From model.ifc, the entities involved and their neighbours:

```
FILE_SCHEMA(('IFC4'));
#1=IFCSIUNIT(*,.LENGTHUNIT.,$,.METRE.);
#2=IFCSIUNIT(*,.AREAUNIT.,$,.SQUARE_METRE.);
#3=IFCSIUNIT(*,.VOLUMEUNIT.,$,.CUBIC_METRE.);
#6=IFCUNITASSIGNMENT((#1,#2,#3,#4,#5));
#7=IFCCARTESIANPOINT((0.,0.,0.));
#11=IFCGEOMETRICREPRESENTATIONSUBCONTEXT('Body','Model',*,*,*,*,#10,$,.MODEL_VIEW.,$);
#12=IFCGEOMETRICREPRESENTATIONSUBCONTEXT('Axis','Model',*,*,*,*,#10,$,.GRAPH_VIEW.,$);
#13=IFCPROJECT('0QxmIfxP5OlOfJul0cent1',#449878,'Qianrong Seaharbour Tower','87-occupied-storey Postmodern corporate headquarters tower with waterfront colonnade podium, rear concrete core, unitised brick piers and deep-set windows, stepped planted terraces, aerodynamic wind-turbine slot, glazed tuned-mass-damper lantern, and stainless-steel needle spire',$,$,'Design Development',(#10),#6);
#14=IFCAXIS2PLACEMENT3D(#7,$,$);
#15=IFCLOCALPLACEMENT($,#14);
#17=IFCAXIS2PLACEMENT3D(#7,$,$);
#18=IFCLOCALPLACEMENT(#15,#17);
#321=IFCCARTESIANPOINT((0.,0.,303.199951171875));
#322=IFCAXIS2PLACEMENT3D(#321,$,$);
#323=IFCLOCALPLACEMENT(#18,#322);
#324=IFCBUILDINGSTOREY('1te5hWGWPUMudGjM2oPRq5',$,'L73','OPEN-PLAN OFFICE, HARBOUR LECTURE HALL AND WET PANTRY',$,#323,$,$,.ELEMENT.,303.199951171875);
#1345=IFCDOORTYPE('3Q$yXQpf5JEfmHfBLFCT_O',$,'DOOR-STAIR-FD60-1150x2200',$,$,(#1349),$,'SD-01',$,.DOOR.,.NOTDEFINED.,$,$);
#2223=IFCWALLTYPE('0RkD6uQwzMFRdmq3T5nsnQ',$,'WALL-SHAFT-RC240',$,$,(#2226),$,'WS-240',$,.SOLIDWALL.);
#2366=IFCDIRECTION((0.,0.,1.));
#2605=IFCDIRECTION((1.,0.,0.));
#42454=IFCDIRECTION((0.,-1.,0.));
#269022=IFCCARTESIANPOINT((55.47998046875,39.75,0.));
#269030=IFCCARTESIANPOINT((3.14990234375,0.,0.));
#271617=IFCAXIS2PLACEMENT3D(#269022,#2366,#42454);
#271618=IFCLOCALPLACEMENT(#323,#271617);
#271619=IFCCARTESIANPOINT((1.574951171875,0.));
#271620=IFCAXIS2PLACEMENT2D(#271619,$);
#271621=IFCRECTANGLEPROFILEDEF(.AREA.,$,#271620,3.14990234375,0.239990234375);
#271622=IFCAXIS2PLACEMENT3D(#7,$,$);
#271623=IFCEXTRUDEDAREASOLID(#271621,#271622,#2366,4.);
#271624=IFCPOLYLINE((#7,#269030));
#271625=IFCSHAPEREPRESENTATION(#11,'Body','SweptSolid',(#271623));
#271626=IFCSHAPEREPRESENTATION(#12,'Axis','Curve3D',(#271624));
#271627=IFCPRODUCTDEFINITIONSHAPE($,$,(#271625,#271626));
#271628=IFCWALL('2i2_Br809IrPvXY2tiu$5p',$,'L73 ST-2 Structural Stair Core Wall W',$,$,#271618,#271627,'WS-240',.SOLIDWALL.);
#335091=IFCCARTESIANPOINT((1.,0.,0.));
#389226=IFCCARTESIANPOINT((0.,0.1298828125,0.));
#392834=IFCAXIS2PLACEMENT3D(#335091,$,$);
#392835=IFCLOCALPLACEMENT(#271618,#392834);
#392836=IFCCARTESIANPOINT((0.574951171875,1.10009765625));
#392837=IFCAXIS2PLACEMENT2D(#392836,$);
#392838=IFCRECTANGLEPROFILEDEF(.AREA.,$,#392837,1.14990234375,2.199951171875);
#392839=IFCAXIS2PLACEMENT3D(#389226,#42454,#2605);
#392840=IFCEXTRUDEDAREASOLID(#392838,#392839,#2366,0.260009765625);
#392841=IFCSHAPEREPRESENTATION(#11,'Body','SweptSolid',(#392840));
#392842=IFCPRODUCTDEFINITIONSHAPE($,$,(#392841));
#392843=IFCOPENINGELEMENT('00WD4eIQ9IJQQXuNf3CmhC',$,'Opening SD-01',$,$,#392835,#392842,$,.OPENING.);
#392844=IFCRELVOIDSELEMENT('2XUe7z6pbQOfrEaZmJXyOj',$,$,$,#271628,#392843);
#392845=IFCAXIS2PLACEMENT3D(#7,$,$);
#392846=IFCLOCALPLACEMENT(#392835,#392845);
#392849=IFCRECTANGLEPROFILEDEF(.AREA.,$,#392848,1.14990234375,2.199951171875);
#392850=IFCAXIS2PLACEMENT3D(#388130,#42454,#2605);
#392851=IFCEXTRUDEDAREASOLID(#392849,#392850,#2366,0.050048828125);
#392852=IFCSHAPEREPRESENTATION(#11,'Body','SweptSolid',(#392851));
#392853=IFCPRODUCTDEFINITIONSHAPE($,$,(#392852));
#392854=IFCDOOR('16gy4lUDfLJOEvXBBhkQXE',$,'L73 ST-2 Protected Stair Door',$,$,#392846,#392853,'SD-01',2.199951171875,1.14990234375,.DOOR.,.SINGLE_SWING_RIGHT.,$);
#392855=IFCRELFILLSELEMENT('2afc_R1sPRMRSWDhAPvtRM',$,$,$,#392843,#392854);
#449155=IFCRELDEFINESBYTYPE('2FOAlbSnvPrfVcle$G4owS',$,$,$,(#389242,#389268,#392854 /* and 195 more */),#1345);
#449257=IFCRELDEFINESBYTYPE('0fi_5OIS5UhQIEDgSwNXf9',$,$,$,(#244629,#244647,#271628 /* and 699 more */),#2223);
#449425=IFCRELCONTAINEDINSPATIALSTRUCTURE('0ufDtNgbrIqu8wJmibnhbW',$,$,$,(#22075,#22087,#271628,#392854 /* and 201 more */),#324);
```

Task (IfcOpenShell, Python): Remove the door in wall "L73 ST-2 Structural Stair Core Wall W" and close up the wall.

```python
import ifcopenshell
import ifcopenshell.api.feature
import ifcopenshell.api.root
import ifcopenshell.geom
import ifcopenshell.util.shape

model = ifcopenshell.open("model.ifc")
settings = ifcopenshell.geom.settings()


def volume(element):
    """Net volume in cubic metres, openings subtracted."""
    shape = ifcopenshell.geom.create_shape(settings, element)
    return ifcopenshell.util.shape.get_volume(shape.geometry)


door = model.by_id(392854)
opening = door.FillsVoids[0].RelatingOpeningElement
wall = opening.VoidsElements[0].RelatingBuildingElement
before = volume(wall)

ifcopenshell.api.root.remove_product(model, product=door)
ifcopenshell.api.feature.remove_feature(model, feature=opening)

after = volume(wall)

print(f"wall volume {before:.3f} -> {after:.3f} m3")

model.write("model_v2.ifc")
```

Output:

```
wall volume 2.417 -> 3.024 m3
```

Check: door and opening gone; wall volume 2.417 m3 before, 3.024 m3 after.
